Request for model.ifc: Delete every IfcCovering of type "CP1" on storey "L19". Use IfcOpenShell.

First a look at what the model holds.

```python
import ifcopenshell
import ifcopenshell.util.element

model = ifcopenshell.open("model.ifc")
print(model.schema)
storey = next(s for s in model.by_type("IfcBuildingStorey") if s.Name == "L19")
coverings = [e for e in ifcopenshell.util.element.get_decomposition(storey) if e.is_a("IfcCovering")]
seen = {}
for e in coverings:
    element_type = ifcopenshell.util.element.get_type(e)
    name = element_type.Name if element_type not in (None, e) else None
    seen[name] = seen.get(name, 0) + 1
for name, count in sorted(seen.items(), key=str):
    print(count, "x", name)
```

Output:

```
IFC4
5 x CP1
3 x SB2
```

```python
import ifcopenshell
import ifcopenshell.api.root
import ifcopenshell.util.element

model = ifcopenshell.open("model.ifc")

storey = next(s for s in model.by_type("IfcBuildingStorey") if s.Name == "L19")
coverings = [e for e in ifcopenshell.util.element.get_decomposition(storey) if e.is_a("IfcCovering")]
targets = [e for e in coverings if (t := ifcopenshell.util.element.get_type(e)) not in (None, e) and t.Name == "CP1"]

for e in targets:
    ifcopenshell.api.root.remove_product(model, product=e)
print(len(targets), "removed")

model.write("model_edited.ifc")
```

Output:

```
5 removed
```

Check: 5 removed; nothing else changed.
